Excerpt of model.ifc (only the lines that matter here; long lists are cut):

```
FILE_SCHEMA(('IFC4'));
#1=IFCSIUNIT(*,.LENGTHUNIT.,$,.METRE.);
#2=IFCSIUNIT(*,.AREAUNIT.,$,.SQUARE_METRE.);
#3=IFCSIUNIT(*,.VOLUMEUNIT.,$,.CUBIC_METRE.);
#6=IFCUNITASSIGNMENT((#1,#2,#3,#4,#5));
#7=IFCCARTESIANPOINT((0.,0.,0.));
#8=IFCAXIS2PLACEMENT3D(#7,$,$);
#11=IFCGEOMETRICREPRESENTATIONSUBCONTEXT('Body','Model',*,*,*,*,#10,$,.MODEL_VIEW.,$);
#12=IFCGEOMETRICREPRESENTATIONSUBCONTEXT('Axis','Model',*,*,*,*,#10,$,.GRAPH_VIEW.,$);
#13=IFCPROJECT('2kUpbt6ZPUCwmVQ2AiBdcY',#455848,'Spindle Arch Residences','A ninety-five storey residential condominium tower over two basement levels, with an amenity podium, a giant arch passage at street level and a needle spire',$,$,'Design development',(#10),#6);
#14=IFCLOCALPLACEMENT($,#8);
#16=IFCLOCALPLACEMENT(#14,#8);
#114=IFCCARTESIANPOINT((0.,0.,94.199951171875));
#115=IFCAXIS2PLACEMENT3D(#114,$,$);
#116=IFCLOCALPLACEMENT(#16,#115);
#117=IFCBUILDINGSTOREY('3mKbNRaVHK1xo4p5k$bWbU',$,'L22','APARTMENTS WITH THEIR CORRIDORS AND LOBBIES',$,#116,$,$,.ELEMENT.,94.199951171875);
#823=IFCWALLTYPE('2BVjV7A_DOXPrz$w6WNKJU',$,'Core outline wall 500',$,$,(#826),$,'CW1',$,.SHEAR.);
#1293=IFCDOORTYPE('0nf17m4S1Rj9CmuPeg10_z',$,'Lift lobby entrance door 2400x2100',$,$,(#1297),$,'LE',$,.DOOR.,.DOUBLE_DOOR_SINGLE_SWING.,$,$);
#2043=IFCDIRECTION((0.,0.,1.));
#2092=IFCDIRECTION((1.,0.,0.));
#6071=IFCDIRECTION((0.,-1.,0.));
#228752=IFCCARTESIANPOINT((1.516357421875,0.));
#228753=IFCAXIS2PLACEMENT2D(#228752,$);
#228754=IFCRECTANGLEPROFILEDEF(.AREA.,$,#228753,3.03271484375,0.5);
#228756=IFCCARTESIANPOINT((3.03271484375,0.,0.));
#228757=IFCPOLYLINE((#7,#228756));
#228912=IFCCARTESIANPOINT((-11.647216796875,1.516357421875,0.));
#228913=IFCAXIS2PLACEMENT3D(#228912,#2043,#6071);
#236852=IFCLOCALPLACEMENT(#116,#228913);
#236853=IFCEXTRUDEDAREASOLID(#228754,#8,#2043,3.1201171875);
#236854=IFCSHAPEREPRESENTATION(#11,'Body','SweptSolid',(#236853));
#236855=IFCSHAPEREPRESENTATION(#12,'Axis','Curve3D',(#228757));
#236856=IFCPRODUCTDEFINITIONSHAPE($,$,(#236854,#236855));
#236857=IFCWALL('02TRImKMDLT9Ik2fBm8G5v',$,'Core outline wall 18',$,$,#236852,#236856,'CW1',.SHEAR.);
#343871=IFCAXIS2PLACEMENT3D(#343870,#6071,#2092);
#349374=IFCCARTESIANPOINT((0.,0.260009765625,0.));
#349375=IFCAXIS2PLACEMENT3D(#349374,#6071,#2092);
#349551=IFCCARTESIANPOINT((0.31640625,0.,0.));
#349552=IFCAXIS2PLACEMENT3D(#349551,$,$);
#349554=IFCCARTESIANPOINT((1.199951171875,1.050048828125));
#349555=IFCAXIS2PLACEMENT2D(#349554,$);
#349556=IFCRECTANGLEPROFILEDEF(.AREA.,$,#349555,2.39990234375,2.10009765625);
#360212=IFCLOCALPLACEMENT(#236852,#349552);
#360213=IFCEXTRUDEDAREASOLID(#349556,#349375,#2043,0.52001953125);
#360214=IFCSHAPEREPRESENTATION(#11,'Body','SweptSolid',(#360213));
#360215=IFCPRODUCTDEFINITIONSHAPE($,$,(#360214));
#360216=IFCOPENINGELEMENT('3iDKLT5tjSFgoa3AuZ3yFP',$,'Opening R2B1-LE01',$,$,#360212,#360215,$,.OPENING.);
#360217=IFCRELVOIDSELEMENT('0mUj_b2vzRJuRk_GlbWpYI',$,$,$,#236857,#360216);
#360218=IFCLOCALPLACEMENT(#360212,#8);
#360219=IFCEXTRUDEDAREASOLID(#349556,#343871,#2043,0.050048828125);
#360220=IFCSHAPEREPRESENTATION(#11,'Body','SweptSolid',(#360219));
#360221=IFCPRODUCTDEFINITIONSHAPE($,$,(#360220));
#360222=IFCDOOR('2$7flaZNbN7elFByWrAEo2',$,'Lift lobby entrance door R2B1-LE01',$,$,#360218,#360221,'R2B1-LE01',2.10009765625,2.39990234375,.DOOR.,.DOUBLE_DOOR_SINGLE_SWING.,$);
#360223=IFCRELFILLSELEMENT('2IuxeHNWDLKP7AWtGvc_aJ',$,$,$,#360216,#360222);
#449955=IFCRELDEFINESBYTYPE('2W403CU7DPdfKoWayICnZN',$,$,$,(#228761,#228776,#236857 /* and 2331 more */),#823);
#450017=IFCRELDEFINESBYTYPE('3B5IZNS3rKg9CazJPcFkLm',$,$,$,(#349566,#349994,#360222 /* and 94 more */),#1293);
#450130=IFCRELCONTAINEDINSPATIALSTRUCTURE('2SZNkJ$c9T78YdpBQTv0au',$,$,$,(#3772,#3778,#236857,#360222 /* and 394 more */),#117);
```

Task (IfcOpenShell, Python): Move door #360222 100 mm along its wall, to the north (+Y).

```python
import ifcopenshell
import ifcopenshell.api.geometry
import ifcopenshell.util.placement

model = ifcopenshell.open("model.ifc")

door = model.by_guid("2$7flaZNbN7elFByWrAEo2")
opening = door.FillsVoids[0].RelatingOpeningElement
wall = opening.VoidsElements[0].RelatingBuildingElement

wall_matrix = ifcopenshell.util.placement.get_local_placement(wall.ObjectPlacement)
shift = wall_matrix[:3, 0] * -0.1
before = ifcopenshell.util.placement.get_local_placement(door.ObjectPlacement)[:3, 3].copy()

# The door is placed relative to its opening, so it follows when the opening moves.
matrix = ifcopenshell.util.placement.get_local_placement(opening.ObjectPlacement)
matrix[:3, 3] += shift
ifcopenshell.api.geometry.edit_object_placement(
    model, product=opening, matrix=matrix, is_si=False, should_transform_children=True
)

after = ifcopenshell.util.placement.get_local_placement(door.ObjectPlacement)[:3, 3]
print("door moved by", (after - before).round(3) + 0.0)

model.write("model-out.ifc")
```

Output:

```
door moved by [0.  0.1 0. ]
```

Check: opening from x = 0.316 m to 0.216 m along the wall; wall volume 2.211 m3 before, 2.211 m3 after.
